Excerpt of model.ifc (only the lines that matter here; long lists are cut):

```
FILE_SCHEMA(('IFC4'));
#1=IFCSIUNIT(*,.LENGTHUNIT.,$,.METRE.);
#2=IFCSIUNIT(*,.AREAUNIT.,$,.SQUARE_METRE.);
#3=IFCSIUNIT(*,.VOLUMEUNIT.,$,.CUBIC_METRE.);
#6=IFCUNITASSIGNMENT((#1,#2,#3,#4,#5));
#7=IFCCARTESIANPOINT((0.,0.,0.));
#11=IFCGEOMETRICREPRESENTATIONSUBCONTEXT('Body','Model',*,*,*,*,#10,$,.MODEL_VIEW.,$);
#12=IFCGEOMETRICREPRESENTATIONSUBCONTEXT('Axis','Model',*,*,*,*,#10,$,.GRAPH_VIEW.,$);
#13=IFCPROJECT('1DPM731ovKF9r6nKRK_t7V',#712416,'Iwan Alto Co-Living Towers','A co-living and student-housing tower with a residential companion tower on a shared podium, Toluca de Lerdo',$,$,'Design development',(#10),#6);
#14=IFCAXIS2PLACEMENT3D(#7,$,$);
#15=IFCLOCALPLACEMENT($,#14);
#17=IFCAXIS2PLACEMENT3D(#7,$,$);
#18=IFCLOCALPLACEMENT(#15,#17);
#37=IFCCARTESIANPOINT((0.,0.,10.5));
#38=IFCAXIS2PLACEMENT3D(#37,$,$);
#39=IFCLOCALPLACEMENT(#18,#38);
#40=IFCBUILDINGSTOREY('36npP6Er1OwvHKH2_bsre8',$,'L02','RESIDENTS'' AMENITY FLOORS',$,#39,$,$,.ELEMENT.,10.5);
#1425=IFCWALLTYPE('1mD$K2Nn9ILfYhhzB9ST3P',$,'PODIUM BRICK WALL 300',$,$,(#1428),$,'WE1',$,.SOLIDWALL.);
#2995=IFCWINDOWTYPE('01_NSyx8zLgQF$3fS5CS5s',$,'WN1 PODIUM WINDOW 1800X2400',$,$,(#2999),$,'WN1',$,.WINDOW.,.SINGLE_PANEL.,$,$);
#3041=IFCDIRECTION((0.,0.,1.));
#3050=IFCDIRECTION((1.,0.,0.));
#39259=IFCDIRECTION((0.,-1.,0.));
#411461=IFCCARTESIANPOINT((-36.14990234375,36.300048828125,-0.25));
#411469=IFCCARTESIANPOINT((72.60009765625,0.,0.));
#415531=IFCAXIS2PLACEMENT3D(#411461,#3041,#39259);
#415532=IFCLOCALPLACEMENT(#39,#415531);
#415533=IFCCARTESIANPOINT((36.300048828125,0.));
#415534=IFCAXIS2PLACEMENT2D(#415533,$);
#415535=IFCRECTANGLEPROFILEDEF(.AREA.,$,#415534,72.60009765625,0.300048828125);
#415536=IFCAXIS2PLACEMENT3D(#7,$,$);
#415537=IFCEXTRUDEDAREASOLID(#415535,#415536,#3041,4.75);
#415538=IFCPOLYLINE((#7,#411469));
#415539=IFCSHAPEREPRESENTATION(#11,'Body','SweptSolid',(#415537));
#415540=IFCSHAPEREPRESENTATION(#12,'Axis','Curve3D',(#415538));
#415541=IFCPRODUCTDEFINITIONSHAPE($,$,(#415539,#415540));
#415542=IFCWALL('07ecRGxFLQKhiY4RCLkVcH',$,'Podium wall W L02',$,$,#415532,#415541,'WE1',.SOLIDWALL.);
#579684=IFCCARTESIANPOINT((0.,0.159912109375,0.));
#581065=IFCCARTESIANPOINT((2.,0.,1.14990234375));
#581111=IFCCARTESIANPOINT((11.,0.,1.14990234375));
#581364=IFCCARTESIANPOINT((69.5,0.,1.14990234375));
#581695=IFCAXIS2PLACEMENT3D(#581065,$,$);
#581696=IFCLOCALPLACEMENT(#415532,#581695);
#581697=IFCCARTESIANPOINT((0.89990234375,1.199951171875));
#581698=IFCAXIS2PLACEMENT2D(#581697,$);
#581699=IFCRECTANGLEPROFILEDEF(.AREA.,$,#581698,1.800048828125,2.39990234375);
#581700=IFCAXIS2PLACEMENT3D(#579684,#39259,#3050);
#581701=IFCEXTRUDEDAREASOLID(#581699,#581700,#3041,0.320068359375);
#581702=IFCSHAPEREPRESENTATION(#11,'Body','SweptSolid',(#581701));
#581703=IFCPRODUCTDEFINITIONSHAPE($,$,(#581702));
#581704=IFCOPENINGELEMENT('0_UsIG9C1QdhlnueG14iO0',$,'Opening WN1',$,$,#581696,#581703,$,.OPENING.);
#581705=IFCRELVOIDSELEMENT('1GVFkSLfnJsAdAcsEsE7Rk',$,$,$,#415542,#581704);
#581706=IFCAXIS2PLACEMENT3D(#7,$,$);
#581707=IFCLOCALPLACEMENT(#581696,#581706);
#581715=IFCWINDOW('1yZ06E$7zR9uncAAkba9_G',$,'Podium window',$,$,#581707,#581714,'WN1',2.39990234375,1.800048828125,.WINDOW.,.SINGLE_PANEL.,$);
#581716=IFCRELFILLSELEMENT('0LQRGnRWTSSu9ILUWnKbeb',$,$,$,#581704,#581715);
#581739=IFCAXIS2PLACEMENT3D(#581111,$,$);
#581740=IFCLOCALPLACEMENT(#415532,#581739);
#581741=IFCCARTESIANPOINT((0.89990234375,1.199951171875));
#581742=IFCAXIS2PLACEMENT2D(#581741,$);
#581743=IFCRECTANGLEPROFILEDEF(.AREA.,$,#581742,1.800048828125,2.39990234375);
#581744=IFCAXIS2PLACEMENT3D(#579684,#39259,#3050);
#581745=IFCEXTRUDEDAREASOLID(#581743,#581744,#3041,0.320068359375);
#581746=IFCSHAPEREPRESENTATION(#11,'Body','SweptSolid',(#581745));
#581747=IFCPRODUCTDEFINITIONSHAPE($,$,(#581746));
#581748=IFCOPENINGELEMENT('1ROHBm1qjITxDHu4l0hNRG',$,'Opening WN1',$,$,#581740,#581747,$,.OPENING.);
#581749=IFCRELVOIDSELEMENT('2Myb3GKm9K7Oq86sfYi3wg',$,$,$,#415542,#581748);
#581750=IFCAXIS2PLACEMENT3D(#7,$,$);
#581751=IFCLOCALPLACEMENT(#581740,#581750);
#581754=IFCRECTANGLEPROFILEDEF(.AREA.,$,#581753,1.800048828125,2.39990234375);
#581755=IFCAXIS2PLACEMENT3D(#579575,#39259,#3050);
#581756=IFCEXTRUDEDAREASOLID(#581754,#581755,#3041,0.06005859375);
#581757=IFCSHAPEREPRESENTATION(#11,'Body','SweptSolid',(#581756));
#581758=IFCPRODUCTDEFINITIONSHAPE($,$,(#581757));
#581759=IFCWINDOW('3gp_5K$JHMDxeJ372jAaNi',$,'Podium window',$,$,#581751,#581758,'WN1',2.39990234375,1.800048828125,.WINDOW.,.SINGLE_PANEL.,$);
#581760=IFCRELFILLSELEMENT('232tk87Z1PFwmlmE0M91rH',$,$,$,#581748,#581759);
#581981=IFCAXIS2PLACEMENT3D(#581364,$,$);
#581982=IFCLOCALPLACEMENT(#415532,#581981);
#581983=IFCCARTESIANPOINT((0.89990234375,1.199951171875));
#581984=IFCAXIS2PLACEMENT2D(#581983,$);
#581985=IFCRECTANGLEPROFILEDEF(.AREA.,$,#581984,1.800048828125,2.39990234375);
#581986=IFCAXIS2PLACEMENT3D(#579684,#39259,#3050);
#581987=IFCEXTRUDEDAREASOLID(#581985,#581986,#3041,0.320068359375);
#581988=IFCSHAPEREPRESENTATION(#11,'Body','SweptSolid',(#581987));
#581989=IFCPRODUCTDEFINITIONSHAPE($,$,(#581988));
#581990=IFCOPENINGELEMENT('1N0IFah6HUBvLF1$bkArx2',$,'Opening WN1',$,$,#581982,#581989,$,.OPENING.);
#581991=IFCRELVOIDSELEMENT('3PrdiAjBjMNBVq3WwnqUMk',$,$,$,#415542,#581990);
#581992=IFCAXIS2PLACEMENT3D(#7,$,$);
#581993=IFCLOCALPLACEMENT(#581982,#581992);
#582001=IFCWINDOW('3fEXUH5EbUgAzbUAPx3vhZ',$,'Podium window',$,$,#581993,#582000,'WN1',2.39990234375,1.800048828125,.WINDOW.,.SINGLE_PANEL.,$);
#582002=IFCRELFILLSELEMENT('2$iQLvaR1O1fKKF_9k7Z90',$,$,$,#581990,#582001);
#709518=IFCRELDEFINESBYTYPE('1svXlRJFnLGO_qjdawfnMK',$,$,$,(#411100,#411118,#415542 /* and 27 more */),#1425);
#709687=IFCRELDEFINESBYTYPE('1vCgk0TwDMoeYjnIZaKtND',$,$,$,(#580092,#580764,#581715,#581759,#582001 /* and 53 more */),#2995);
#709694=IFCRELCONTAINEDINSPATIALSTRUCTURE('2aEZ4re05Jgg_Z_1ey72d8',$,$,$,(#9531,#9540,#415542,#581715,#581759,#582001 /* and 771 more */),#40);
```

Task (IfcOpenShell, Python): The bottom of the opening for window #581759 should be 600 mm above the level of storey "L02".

```python
import numpy as np
import ifcopenshell
import ifcopenshell.api.geometry
import ifcopenshell.geom
import ifcopenshell.util.element
import ifcopenshell.util.placement
import ifcopenshell.util.shape
import ifcopenshell.util.unit

model = ifcopenshell.open("model.ifc")
unit_scale = ifcopenshell.util.unit.calculate_unit_scale(model)

window = model.by_id(581759)
opening = window.FillsVoids[0].RelatingOpeningElement
storey = ifcopenshell.util.element.get_container(window, ifc_class="IfcBuildingStorey")
level = ifcopenshell.util.placement.get_local_placement(storey.ObjectPlacement)[2, 3]

# The opening's origin need not be at the sill, so measure its lowest point.
shape = ifcopenshell.geom.create_shape(ifcopenshell.geom.settings(), opening)
bottom = ifcopenshell.util.shape.get_shape_bottom_elevation(shape, shape.geometry) / unit_scale
dz = level + 0.6 - bottom

shift = np.array([0.0, 0.0, dz])
# The window is placed relative to its opening, so it follows when the opening moves.
matrix = ifcopenshell.util.placement.get_local_placement(opening.ObjectPlacement)
matrix[:3, 3] += shift
ifcopenshell.api.geometry.edit_object_placement(
    model, product=opening, matrix=matrix, is_si=False, should_transform_children=True
)

print(f"moved by {dz * unit_scale:+.3f} m")

model.write("model_v2.ifc")
```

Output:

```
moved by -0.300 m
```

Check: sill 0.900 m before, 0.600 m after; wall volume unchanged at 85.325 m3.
